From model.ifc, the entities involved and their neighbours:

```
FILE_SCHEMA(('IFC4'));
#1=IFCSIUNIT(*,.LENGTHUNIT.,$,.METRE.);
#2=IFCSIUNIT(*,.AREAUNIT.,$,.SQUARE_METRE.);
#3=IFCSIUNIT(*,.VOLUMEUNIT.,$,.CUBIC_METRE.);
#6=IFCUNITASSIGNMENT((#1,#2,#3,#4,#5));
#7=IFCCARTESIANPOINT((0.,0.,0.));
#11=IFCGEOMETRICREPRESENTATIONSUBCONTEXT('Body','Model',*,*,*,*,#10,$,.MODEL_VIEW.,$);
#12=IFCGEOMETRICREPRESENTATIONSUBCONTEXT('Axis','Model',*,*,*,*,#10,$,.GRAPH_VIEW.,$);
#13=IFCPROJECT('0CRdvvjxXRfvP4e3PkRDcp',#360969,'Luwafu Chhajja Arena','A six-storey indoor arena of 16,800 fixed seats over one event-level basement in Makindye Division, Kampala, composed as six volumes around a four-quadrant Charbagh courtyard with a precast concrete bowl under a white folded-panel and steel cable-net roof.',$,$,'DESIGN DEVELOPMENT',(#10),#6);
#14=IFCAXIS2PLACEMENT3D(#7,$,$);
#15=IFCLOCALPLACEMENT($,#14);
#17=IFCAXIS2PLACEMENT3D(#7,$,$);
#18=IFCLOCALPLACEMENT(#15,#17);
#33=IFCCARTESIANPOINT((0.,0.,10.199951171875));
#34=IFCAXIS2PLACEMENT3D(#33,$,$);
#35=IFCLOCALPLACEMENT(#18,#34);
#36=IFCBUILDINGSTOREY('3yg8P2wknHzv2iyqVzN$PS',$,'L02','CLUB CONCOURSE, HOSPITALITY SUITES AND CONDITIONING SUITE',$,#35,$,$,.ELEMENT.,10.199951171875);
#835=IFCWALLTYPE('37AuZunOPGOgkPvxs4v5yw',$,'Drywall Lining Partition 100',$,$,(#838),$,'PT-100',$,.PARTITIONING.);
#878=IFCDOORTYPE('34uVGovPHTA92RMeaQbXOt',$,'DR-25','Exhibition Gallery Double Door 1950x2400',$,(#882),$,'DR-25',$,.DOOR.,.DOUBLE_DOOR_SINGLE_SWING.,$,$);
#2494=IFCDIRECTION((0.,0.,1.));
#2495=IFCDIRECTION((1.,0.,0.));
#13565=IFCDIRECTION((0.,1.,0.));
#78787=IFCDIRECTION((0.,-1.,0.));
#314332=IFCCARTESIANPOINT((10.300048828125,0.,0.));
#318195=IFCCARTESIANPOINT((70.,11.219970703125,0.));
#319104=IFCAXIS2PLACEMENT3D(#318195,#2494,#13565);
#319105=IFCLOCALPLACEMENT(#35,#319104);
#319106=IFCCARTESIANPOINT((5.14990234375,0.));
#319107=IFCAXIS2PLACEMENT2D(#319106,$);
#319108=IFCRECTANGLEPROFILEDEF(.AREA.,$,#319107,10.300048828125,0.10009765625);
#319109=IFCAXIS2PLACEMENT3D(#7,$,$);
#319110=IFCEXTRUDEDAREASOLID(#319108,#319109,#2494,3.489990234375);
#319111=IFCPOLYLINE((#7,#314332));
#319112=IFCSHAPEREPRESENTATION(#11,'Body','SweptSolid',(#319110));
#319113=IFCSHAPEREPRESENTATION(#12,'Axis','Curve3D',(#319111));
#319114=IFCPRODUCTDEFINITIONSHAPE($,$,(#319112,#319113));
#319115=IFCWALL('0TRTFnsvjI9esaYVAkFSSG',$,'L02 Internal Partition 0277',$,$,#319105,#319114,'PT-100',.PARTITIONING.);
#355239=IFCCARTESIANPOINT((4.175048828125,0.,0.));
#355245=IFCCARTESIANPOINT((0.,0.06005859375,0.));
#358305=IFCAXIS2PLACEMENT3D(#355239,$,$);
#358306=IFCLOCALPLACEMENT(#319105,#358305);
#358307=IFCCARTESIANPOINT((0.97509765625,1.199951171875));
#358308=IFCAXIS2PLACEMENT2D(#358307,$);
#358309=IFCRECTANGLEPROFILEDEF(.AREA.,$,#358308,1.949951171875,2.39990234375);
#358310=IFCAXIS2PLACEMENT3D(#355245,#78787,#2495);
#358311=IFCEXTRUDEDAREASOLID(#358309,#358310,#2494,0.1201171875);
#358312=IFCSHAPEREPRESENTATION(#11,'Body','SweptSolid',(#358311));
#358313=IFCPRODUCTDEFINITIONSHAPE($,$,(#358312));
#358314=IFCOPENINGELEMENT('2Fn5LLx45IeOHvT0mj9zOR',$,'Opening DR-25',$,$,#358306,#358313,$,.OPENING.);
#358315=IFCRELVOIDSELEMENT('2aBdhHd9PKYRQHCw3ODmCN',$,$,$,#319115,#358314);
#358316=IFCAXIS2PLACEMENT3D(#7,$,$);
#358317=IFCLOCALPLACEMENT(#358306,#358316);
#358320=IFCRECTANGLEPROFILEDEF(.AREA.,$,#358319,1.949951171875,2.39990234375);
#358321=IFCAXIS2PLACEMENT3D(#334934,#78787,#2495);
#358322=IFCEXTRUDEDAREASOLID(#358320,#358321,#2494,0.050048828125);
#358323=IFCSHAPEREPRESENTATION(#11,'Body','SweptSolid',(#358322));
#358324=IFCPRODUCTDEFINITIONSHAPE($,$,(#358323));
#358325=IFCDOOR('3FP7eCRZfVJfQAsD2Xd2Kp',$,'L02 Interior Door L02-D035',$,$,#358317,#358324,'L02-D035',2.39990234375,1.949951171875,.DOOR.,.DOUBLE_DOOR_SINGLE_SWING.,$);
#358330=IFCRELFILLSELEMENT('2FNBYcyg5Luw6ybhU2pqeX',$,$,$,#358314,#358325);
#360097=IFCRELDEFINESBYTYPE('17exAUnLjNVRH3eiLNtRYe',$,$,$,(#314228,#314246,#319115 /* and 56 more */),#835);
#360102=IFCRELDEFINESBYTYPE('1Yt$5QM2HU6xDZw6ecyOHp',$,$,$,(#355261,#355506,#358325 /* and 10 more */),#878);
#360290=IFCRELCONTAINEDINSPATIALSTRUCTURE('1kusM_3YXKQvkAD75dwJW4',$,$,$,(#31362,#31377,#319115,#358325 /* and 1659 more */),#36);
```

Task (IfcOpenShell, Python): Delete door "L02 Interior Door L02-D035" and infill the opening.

```python
import ifcopenshell
import ifcopenshell.api.feature
import ifcopenshell.api.root
import ifcopenshell.geom
import ifcopenshell.util.shape

model = ifcopenshell.open("model.ifc")
settings = ifcopenshell.geom.settings()


def volume(element):
    """Net volume in cubic metres, openings subtracted."""
    shape = ifcopenshell.geom.create_shape(settings, element)
    return ifcopenshell.util.shape.get_volume(shape.geometry)


door = model.by_guid("3FP7eCRZfVJfQAsD2Xd2Kp")
opening = door.FillsVoids[0].RelatingOpeningElement
wall = opening.VoidsElements[0].RelatingBuildingElement
before = volume(wall)

ifcopenshell.api.root.remove_product(model, product=door)
ifcopenshell.api.feature.remove_feature(model, feature=opening)

after = volume(wall)

print(f"wall volume {before:.3f} -> {after:.3f} m3")

model.write("model_edited.ifc")
```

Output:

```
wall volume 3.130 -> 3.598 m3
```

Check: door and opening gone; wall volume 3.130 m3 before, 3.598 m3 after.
